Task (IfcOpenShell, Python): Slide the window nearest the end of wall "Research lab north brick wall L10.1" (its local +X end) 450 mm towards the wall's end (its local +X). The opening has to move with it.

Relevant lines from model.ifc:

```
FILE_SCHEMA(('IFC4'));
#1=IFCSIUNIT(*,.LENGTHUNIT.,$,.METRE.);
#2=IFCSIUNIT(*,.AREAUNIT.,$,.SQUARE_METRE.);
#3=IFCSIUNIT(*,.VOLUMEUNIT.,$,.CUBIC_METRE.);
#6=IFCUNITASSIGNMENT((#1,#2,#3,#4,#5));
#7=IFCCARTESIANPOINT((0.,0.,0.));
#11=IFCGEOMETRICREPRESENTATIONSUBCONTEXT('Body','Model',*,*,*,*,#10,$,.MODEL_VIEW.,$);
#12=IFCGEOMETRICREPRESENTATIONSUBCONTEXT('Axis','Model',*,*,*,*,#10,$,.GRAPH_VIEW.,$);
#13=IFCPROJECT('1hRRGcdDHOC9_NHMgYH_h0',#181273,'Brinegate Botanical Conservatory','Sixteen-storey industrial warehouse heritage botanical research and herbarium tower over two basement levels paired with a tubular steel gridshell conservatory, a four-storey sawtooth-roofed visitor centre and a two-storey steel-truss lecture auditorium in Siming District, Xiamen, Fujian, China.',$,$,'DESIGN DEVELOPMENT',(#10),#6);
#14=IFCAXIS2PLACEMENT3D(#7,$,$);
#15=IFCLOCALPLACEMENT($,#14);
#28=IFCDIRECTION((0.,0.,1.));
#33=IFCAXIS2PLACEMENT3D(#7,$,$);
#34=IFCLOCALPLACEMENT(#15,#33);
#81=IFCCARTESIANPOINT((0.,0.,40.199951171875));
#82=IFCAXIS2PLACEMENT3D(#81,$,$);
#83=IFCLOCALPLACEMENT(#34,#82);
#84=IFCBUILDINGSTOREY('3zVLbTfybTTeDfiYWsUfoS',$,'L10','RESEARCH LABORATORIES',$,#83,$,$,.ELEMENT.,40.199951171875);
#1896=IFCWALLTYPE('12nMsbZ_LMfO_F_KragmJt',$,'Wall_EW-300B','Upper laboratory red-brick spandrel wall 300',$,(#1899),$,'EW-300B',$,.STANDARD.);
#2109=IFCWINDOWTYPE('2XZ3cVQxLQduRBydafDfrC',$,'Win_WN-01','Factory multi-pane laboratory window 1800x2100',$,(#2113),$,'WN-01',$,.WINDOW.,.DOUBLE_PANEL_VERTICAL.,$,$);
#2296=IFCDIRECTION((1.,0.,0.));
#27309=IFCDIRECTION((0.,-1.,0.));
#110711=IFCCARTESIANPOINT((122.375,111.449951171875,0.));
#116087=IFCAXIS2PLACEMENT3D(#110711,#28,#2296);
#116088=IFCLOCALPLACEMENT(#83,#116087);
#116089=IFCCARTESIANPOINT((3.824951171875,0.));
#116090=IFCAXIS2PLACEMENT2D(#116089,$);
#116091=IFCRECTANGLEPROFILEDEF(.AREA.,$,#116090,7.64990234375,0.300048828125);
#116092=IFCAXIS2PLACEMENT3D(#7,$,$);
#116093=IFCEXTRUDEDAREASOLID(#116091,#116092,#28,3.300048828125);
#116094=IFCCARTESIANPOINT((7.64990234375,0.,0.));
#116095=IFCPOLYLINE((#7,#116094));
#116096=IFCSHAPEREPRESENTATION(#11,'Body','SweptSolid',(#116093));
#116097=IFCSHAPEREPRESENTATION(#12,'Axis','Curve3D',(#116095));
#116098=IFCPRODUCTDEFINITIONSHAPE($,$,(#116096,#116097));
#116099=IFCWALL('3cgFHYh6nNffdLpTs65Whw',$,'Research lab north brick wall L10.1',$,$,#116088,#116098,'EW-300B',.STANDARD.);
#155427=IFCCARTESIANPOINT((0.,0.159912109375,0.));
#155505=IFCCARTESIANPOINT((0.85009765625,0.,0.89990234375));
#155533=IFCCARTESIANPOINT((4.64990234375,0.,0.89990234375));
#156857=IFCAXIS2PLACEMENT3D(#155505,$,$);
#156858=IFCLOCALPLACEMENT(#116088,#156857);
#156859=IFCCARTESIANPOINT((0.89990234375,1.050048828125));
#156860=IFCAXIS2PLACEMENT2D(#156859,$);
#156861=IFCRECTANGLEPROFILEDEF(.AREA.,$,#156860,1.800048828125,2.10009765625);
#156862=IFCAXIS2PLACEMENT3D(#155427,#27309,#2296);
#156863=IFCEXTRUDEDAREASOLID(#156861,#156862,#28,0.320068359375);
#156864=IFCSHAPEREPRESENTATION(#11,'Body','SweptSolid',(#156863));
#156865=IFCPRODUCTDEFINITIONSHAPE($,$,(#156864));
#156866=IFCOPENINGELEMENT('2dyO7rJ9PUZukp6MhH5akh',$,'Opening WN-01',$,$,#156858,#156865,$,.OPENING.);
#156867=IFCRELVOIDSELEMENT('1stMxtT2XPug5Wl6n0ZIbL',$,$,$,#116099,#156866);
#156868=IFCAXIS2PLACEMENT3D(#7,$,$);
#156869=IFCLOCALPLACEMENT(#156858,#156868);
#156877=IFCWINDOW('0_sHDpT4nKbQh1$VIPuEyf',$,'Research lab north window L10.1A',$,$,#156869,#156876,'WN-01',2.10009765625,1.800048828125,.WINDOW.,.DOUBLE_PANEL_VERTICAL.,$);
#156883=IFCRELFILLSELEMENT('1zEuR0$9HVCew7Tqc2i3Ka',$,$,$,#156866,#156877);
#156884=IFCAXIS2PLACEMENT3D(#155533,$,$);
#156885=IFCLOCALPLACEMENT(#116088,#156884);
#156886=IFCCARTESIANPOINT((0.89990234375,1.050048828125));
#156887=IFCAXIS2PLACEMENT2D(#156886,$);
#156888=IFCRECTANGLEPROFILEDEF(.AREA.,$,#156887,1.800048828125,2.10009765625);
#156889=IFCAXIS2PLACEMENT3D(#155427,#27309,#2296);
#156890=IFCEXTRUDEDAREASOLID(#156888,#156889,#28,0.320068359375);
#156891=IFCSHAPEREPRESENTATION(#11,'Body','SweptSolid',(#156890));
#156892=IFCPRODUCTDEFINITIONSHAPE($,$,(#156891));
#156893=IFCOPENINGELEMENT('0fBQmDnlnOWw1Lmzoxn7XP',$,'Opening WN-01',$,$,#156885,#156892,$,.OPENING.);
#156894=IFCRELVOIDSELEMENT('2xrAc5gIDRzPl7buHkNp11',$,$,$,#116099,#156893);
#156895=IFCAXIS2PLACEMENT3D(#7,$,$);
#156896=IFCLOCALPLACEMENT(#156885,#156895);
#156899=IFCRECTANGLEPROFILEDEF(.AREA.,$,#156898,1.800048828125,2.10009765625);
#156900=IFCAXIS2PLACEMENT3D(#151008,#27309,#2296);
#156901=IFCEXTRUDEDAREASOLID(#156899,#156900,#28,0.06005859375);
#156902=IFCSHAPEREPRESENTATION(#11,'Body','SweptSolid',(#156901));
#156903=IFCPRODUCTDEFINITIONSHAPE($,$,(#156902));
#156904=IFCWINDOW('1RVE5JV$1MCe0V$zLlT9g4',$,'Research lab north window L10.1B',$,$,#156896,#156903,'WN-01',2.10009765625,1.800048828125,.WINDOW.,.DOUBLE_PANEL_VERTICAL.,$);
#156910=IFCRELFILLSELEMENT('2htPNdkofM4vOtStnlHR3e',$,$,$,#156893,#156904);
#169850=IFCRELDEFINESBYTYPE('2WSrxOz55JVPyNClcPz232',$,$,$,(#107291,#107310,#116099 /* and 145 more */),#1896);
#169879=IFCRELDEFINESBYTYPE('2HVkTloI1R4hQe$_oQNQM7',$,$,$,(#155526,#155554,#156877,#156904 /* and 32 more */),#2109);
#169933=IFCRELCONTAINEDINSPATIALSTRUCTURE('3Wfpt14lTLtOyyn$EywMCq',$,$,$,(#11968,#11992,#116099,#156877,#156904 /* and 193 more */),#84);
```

```python
import ifcopenshell
import ifcopenshell.api.geometry
import ifcopenshell.util.placement

model = ifcopenshell.open("model.ifc")

window = model.by_guid("1RVE5JV$1MCe0V$zLlT9g4")
opening = window.FillsVoids[0].RelatingOpeningElement
wall = opening.VoidsElements[0].RelatingBuildingElement

wall_matrix = ifcopenshell.util.placement.get_local_placement(wall.ObjectPlacement)
shift = wall_matrix[:3, 0] * 0.45
before = ifcopenshell.util.placement.get_local_placement(window.ObjectPlacement)[:3, 3].copy()

# The window is placed relative to its opening, so it follows when the opening moves.
matrix = ifcopenshell.util.placement.get_local_placement(opening.ObjectPlacement)
matrix[:3, 3] += shift
ifcopenshell.api.geometry.edit_object_placement(
    model, product=opening, matrix=matrix, is_si=False, should_transform_children=True
)

after = ifcopenshell.util.placement.get_local_placement(window.ObjectPlacement)[:3, 3]
print("window moved by", (after - before).round(3) + 0.0)

model.write("model-out.ifc")
```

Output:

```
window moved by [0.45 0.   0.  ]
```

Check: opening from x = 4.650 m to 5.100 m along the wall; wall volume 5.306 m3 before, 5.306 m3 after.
